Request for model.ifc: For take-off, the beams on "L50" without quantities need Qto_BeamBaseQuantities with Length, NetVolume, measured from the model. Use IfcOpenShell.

First a look at what the model holds.

```python
import ifcopenshell
import ifcopenshell.util.element
import ifcopenshell.util.unit

model = ifcopenshell.open("model.ifc")
print(model.schema)
for unit_type in ("LENGTHUNIT", "AREAUNIT", "VOLUMEUNIT"):
    print(unit_type, ifcopenshell.util.unit.calculate_unit_scale(model, unit_type))
storey = next(s for s in model.by_type("IfcBuildingStorey") if s.Name == "L50")
beams = [e for e in ifcopenshell.util.element.get_decomposition(storey) if e.is_a("IfcBeam")]
for e in sorted(beams, key=lambda e: e.id()):
    print(e.id(), e.is_a(), e.Name, list(ifcopenshell.util.element.get_psets(e, qtos_only=True)), sep=" | ")
```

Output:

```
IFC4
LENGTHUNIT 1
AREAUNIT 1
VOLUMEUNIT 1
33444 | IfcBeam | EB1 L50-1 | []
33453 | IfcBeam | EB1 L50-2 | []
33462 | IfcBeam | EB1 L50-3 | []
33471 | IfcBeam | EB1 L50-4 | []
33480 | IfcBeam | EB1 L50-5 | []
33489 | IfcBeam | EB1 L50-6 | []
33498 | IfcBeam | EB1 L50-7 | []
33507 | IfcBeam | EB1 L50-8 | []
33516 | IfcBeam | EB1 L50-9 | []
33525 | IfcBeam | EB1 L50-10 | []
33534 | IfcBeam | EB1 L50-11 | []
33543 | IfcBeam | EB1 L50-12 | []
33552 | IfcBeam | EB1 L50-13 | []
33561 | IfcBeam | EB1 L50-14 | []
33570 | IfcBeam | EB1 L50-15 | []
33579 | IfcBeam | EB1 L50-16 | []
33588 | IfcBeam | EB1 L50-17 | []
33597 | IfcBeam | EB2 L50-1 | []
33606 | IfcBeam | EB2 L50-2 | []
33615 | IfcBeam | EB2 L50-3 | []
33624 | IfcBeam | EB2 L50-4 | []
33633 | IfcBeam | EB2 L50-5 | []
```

```python
import ifcopenshell
import ifcopenshell.api.pset
import ifcopenshell.geom
import ifcopenshell.util.element
import ifcopenshell.util.shape
import ifcopenshell.util.unit

model = ifcopenshell.open("model.ifc")
unit_scale = ifcopenshell.util.unit.calculate_unit_scale(model)
volume_scale = ifcopenshell.util.unit.calculate_unit_scale(model, "VOLUMEUNIT")
settings = ifcopenshell.geom.settings()

storey = next(s for s in model.by_type("IfcBuildingStorey") if s.Name == "L50")
beams = [e for e in ifcopenshell.util.element.get_decomposition(storey) if e.is_a("IfcBeam")]

for e in sorted(beams, key=lambda e: e.id()):
    if ifcopenshell.util.element.get_psets(e, qtos_only=True, should_inherit=False):
        continue
    # Geometry comes back in metres, in the element's own axes.
    shape = ifcopenshell.geom.create_shape(settings, e)
    values = {
        "Length": ifcopenshell.util.shape.get_max_xyz(shape.geometry) / unit_scale,
        "NetVolume": ifcopenshell.util.shape.get_volume(shape.geometry) / volume_scale,
    }
    qto = ifcopenshell.api.pset.add_qto(model, product=e, name="Qto_BeamBaseQuantities")
    ifcopenshell.api.pset.edit_qto(model, qto=qto, properties=values)
    print(e.id(), {k: round(v, 3) for k, v in values.items()})

model.write("model_edited.ifc")
```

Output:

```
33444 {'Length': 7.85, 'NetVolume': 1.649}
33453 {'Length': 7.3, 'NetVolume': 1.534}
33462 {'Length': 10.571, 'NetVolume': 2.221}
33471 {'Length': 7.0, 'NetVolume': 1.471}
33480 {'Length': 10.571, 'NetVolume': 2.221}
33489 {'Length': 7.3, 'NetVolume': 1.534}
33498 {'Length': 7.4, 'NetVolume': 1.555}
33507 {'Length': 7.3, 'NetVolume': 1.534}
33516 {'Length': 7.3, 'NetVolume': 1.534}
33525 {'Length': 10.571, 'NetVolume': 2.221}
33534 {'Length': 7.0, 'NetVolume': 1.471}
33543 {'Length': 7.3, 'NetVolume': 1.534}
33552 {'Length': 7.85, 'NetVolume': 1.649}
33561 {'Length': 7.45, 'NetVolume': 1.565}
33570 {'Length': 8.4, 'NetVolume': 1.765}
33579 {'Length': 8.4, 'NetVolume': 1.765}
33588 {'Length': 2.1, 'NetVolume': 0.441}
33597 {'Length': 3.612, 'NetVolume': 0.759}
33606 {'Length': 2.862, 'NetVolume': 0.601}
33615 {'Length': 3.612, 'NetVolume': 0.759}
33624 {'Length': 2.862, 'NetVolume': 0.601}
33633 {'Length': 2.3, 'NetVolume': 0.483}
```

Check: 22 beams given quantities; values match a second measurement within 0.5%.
